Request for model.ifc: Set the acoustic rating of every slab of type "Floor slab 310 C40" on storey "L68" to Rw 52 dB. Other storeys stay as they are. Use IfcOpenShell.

First a look at what the model holds.

```python
import ifcopenshell
import ifcopenshell.util.element

model = ifcopenshell.open("model.ifc")
print(model.schema)
storey = next(s for s in model.by_type("IfcBuildingStorey") if s.Name == "L68")
slabs = [e for e in ifcopenshell.util.element.get_decomposition(storey) if e.is_a("IfcSlab")]
seen = {}
for e in slabs:
    element_type = ifcopenshell.util.element.get_type(e)
    key = (element_type.Name if element_type != e and element_type else None, ifcopenshell.util.element.get_pset(e, "Pset_SlabCommon", "AcousticRating"))
    seen[key] = seen.get(key, 0) + 1
for (name, value), count in sorted(seen.items(), key=str):
    print(count, "x", name, "|", value)
```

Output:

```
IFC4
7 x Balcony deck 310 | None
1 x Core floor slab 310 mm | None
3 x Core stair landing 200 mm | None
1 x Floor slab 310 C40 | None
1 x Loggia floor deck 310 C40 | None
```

```python
import ifcopenshell
import ifcopenshell.api.pset
import ifcopenshell.util.element

model = ifcopenshell.open("model.ifc")

storey = next(s for s in model.by_type("IfcBuildingStorey") if s.Name == "L68")
slabs = [e for e in ifcopenshell.util.element.get_decomposition(storey) if e.is_a("IfcSlab")]

count = 0
for e in slabs:
    element_type = ifcopenshell.util.element.get_type(e)
    if element_type in (None, e) or element_type.Name != "Floor slab 310 C40":
        continue
    found = ifcopenshell.util.element.get_pset(e, "Pset_SlabCommon", should_inherit=False)
    if found:
        pset = model.by_id(found["id"])
        if len(ifcopenshell.util.element.get_elements_by_pset(pset)) > 1:
            pset = ifcopenshell.api.pset.unshare_pset(model, products=[e], pset=pset)[0]
    else:
        pset = ifcopenshell.api.pset.add_pset(model, product=e, name="Pset_SlabCommon")
    ifcopenshell.api.pset.edit_pset(model, pset=pset, properties={"AcousticRating": "Rw 52 dB"})
    count += 1

print(count, "slabs updated")

model.write("model_rev.ifc")
```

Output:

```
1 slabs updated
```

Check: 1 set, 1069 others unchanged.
